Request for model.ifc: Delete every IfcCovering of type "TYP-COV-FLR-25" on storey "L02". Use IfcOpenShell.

First a look at what the model holds.

```python
import ifcopenshell
import ifcopenshell.util.element

model = ifcopenshell.open("model.ifc")
print(model.schema)
storey = next(s for s in model.by_type("IfcBuildingStorey") if s.Name == "L02")
coverings = [e for e in ifcopenshell.util.element.get_decomposition(storey) if e.is_a("IfcCovering")]
seen = {}
for e in coverings:
    element_type = ifcopenshell.util.element.get_type(e)
    name = element_type.Name if element_type not in (None, e) else None
    seen[name] = seen.get(name, 0) + 1
for name, count in sorted(seen.items(), key=str):
    print(count, "x", name)
```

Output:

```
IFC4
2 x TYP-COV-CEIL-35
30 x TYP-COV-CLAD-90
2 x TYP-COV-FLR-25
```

```python
import ifcopenshell
import ifcopenshell.api.root
import ifcopenshell.util.element

model = ifcopenshell.open("model.ifc")

storey = next(s for s in model.by_type("IfcBuildingStorey") if s.Name == "L02")
coverings = [e for e in ifcopenshell.util.element.get_decomposition(storey) if e.is_a("IfcCovering")]
targets = [e for e in coverings if (t := ifcopenshell.util.element.get_type(e)) not in (None, e) and t.Name == "TYP-COV-FLR-25"]

for e in targets:
    ifcopenshell.api.root.remove_product(model, product=e)
print(len(targets), "removed")

model.write("model_v2.ifc")
```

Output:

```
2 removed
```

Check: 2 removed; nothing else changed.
